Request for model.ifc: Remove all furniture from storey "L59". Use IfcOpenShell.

First a look at what the model holds.

```python
import ifcopenshell
import ifcopenshell.util.element

model = ifcopenshell.open("model.ifc")
print(model.schema)
storey = next(s for s in model.by_type("IfcBuildingStorey") if s.Name == "L59")
furniture = [e for e in ifcopenshell.util.element.get_decomposition(storey) if e.is_a("IfcFurnishingElement")]
seen = {}
for e in furniture:
    element_type = ifcopenshell.util.element.get_type(e)
    name = element_type.Name if element_type not in (None, e) else None
    seen[name] = seen.get(name, 0) + 1
for name, count in sorted(seen.items(), key=str):
    print(count, "x", name)
```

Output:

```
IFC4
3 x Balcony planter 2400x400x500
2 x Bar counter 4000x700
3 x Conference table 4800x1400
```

```python
import ifcopenshell
import ifcopenshell.api.root
import ifcopenshell.util.element

model = ifcopenshell.open("model.ifc")

storey = next(s for s in model.by_type("IfcBuildingStorey") if s.Name == "L59")
furniture = [e for e in ifcopenshell.util.element.get_decomposition(storey) if e.is_a("IfcFurnishingElement")]

for e in furniture:
    ifcopenshell.api.root.remove_product(model, product=e)
print(len(furniture), "removed")

model.write("model_edited.ifc")
```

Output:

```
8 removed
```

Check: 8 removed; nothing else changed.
